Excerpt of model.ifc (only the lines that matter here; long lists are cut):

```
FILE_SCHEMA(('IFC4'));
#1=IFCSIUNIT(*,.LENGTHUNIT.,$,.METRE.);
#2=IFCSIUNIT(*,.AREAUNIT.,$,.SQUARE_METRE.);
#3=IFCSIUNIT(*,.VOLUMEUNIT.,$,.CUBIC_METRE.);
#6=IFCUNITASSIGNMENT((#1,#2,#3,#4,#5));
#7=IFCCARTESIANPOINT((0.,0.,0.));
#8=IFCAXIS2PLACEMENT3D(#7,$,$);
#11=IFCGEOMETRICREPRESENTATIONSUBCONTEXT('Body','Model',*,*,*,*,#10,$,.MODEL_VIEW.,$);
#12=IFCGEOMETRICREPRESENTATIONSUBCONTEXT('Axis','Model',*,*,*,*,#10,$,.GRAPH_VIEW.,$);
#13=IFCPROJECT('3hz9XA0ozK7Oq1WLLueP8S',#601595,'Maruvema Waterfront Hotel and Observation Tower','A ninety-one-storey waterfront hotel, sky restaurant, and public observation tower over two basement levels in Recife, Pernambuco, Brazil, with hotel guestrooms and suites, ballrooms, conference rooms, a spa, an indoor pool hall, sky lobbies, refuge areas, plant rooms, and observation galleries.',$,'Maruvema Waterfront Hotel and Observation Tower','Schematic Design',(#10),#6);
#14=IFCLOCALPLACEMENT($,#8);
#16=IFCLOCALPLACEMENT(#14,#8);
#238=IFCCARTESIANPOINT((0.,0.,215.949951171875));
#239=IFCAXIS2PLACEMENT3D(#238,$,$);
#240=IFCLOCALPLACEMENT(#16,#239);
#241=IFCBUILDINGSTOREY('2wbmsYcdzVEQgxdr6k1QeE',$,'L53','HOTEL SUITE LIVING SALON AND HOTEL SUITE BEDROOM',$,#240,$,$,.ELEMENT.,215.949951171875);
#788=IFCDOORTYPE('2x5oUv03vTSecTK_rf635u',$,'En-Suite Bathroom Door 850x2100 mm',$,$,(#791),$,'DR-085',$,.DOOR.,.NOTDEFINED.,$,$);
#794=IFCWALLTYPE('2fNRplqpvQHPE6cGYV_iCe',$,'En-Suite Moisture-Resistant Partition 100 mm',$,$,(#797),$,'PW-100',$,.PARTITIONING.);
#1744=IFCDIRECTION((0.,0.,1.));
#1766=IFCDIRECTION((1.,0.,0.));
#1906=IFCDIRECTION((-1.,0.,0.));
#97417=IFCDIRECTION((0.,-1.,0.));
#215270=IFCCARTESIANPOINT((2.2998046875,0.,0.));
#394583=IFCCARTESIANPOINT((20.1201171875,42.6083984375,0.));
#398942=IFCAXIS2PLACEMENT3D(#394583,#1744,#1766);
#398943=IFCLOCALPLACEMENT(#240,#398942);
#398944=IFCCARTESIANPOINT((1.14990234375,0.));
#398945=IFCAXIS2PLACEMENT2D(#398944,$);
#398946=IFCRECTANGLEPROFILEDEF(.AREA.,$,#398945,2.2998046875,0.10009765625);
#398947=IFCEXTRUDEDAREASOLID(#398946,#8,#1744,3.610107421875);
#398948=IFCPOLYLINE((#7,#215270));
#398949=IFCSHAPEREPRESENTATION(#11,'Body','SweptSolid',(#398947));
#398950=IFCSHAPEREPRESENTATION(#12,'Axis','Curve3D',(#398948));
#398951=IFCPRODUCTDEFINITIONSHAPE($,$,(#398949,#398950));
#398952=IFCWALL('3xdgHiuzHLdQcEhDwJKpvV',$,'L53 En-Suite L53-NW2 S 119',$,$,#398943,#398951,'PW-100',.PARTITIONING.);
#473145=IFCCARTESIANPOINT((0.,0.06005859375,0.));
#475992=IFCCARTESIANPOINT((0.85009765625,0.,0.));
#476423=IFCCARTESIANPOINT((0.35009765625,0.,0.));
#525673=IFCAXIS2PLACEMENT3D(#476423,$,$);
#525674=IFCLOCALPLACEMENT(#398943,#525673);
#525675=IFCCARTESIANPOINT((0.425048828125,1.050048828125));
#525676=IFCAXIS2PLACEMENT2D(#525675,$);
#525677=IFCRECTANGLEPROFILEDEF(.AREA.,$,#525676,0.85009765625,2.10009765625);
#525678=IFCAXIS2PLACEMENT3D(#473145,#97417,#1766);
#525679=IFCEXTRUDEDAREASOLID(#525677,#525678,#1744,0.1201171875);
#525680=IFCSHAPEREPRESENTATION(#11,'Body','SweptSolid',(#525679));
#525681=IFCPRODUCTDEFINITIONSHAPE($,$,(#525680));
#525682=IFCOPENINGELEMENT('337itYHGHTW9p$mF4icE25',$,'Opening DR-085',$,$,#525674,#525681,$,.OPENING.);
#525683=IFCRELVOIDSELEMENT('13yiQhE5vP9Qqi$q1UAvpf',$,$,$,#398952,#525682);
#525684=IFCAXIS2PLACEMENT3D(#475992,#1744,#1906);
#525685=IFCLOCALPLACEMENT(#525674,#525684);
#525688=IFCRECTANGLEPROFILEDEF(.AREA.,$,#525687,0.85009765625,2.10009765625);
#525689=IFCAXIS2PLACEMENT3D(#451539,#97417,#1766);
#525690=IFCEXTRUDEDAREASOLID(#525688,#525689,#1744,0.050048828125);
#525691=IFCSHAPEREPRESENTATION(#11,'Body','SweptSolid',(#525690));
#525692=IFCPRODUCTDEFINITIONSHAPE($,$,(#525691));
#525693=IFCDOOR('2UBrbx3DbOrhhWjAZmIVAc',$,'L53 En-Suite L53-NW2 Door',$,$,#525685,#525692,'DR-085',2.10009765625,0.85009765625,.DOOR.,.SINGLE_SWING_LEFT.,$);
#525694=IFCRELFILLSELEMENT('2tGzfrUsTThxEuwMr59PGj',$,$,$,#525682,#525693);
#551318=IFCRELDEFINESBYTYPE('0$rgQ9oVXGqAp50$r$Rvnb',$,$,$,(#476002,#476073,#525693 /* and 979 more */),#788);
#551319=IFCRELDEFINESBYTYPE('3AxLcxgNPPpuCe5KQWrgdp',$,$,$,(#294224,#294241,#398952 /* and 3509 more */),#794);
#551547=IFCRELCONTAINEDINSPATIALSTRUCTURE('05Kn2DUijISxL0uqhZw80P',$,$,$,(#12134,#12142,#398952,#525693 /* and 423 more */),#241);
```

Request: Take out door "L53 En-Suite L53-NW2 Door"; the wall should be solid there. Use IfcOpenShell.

```python
import ifcopenshell
import ifcopenshell.api.feature
import ifcopenshell.api.root
import ifcopenshell.geom
import ifcopenshell.util.shape

model = ifcopenshell.open("model.ifc")
settings = ifcopenshell.geom.settings()


def volume(element):
    """Net volume in cubic metres, openings subtracted."""
    shape = ifcopenshell.geom.create_shape(settings, element)
    return ifcopenshell.util.shape.get_volume(shape.geometry)


door = model.by_guid("2UBrbx3DbOrhhWjAZmIVAc")
opening = door.FillsVoids[0].RelatingOpeningElement
wall = opening.VoidsElements[0].RelatingBuildingElement
before = volume(wall)

ifcopenshell.api.root.remove_product(model, product=door)
ifcopenshell.api.feature.remove_feature(model, feature=opening)

after = volume(wall)

print(f"wall volume {before:.3f} -> {after:.3f} m3")

model.write("model_v2.ifc")
```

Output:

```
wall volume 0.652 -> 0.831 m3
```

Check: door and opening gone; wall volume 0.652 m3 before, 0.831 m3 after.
